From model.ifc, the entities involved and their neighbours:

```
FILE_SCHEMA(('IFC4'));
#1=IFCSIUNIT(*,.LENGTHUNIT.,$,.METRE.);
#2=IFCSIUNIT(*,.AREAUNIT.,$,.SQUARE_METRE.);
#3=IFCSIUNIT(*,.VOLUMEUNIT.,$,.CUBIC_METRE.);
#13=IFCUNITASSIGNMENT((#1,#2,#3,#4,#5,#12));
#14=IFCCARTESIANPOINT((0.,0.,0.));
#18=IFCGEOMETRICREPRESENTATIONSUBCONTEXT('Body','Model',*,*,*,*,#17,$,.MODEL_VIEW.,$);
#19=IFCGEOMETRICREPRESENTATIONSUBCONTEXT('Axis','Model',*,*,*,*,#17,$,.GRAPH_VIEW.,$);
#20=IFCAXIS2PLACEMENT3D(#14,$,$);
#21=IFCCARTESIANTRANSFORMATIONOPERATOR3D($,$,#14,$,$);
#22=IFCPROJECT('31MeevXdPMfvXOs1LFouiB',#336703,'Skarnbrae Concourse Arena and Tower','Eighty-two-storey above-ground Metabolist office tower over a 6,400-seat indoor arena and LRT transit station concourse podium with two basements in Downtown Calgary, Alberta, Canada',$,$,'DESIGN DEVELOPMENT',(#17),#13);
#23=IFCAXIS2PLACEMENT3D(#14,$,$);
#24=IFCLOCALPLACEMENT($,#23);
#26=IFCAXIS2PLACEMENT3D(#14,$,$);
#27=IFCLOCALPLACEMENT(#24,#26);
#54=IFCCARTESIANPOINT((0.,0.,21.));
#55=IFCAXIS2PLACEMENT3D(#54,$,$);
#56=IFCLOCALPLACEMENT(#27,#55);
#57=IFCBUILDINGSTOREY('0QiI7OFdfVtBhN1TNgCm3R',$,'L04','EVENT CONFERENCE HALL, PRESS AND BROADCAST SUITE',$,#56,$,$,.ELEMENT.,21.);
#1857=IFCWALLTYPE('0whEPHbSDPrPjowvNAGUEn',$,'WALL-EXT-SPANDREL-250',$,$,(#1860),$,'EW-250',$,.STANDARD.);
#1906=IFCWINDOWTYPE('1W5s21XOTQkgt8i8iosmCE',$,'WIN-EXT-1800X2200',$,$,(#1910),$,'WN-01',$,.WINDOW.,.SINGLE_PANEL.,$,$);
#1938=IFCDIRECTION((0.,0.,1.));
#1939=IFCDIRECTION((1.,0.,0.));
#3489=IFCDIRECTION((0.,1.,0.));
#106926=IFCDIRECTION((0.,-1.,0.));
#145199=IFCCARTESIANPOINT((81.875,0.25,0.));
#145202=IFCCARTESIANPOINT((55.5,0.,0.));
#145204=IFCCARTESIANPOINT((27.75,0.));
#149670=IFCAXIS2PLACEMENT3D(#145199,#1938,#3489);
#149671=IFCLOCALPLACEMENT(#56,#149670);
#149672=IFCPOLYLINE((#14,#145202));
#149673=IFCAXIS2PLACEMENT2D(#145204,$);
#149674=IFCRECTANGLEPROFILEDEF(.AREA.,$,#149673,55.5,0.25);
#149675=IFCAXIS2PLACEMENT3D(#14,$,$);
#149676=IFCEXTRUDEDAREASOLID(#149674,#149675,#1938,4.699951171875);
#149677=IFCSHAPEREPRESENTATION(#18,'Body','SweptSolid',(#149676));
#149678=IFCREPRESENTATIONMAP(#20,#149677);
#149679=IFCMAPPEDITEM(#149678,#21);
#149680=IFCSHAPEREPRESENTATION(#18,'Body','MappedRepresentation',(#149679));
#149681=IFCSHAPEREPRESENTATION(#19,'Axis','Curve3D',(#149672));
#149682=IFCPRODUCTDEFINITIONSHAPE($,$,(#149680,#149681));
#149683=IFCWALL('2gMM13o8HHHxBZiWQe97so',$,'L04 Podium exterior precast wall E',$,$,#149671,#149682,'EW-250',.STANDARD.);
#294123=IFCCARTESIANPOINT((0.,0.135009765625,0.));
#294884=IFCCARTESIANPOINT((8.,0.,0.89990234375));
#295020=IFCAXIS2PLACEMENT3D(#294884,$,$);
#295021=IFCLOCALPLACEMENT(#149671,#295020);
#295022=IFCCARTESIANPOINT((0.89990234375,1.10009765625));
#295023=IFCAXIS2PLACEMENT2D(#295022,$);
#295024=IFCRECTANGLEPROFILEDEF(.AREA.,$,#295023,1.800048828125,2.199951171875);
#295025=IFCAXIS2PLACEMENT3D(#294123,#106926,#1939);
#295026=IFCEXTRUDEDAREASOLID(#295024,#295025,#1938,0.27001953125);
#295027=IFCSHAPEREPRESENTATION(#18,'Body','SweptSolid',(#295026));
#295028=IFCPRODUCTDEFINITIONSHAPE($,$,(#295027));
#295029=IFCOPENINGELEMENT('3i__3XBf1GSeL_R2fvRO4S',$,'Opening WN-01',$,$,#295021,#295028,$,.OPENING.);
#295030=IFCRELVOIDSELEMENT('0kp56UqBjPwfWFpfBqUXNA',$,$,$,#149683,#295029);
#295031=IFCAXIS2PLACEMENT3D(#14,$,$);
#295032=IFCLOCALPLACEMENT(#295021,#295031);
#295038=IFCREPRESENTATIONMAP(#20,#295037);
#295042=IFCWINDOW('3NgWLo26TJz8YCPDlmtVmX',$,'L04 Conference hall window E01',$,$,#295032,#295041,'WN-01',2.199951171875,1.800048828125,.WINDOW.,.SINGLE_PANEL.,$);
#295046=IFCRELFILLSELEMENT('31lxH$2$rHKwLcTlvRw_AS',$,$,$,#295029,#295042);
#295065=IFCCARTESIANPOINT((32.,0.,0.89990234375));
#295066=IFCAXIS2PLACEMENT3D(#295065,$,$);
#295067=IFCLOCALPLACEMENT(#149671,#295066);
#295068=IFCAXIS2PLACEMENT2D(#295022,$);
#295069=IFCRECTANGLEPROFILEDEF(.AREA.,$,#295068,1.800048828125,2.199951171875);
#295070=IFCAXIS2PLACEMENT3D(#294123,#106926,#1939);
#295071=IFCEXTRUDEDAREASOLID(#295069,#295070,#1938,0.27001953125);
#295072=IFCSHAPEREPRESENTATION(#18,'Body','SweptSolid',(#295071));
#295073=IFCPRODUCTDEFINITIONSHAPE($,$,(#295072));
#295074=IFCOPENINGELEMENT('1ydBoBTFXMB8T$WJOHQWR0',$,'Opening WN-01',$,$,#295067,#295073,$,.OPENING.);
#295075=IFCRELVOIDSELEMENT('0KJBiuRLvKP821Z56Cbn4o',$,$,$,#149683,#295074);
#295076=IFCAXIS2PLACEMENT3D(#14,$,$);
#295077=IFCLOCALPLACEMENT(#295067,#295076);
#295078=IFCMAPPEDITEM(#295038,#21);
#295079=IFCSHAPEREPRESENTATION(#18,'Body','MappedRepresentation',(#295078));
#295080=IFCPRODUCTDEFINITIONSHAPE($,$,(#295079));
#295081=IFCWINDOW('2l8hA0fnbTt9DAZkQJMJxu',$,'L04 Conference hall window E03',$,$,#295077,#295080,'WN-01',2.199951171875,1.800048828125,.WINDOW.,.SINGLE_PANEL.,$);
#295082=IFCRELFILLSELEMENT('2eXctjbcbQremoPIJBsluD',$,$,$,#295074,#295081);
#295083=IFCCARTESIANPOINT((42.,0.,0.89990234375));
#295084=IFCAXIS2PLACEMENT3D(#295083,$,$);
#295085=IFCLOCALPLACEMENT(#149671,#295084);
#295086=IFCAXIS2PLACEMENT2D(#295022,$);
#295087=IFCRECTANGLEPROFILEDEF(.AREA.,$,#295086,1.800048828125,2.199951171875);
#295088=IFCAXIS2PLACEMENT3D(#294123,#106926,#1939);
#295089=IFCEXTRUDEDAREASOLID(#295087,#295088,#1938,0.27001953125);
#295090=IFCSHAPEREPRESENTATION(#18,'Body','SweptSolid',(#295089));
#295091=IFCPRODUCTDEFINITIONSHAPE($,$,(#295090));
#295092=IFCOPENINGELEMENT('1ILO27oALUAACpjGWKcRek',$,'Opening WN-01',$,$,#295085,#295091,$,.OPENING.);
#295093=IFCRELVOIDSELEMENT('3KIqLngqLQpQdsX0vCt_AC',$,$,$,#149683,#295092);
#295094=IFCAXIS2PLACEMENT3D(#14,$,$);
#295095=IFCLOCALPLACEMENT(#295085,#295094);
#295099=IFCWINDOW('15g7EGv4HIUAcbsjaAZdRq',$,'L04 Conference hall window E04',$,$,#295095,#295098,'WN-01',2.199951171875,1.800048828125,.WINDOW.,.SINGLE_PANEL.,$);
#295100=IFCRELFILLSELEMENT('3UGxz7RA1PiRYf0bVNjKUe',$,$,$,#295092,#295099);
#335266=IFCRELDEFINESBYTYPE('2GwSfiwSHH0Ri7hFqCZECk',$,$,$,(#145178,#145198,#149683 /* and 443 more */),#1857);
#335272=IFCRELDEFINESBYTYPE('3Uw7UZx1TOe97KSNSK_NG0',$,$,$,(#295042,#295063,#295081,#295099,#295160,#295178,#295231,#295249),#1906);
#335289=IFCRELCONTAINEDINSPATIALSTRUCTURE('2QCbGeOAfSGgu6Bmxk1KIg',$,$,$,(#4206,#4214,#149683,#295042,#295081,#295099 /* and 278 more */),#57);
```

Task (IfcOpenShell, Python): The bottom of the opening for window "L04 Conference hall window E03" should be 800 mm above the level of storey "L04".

```python
import numpy as np
import ifcopenshell
import ifcopenshell.api.geometry
import ifcopenshell.geom
import ifcopenshell.util.element
import ifcopenshell.util.placement
import ifcopenshell.util.shape
import ifcopenshell.util.unit

model = ifcopenshell.open("model.ifc")
unit_scale = ifcopenshell.util.unit.calculate_unit_scale(model)

window = model.by_guid("2l8hA0fnbTt9DAZkQJMJxu")
opening = window.FillsVoids[0].RelatingOpeningElement
storey = ifcopenshell.util.element.get_container(window, ifc_class="IfcBuildingStorey")
level = ifcopenshell.util.placement.get_local_placement(storey.ObjectPlacement)[2, 3]

# The opening's origin need not be at the sill, so measure its lowest point.
shape = ifcopenshell.geom.create_shape(ifcopenshell.geom.settings(), opening)
bottom = ifcopenshell.util.shape.get_shape_bottom_elevation(shape, shape.geometry) / unit_scale
dz = level + 0.8 / unit_scale - bottom

shift = np.array([0.0, 0.0, dz])
# The window is placed relative to its opening, so it follows when the opening moves.
matrix = ifcopenshell.util.placement.get_local_placement(opening.ObjectPlacement)
matrix[:3, 3] += shift
ifcopenshell.api.geometry.edit_object_placement(
    model, product=opening, matrix=matrix, is_si=False, should_transform_children=True
)

print(f"moved by {dz * unit_scale:+.3f} m")

model.write("model_rev.ifc")
```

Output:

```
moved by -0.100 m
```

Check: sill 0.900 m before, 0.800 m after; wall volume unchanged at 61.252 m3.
